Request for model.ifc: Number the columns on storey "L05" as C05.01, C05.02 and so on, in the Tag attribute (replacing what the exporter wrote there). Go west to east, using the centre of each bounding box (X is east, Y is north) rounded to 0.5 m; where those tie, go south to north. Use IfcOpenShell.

First a look at what the model holds.

```python
import ifcopenshell
import ifcopenshell.util.element
import ifcopenshell.util.placement

model = ifcopenshell.open("model.ifc")
print(model.schema)
storey = next(s for s in model.by_type("IfcBuildingStorey") if s.Name == "L05")
columns = [e for e in ifcopenshell.util.element.get_decomposition(storey) if e.is_a("IfcColumn")]
for e in sorted(columns, key=lambda e: e.id()):
    origin = ifcopenshell.util.placement.get_local_placement(e.ObjectPlacement)[:3, 3]
    print(e.id(), e.Tag, e.Name, origin.round(2) + 0.0, sep=" | ")
```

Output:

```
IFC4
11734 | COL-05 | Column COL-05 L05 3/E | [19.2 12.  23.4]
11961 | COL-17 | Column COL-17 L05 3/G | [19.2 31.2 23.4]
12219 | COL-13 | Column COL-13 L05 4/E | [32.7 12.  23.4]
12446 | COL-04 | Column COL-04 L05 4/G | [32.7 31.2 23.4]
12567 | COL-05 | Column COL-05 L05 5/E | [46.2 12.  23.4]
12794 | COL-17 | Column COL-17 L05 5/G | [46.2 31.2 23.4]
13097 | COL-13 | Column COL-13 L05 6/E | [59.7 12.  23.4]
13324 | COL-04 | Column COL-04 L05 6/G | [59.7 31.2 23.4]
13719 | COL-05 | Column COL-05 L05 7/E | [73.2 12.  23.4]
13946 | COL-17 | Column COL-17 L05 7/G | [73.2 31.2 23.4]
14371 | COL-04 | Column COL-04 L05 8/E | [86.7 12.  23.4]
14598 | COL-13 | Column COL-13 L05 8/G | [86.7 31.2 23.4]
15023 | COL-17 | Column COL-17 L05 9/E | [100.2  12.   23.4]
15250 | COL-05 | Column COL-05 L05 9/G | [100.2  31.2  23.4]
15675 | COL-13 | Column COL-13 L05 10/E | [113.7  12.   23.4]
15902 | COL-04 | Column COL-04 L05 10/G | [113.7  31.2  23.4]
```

```python
import ifcopenshell
import ifcopenshell.geom
import ifcopenshell.util.element
import ifcopenshell.util.shape

model = ifcopenshell.open("model.ifc")
settings = ifcopenshell.geom.settings()
settings.set("use-world-coords", True)


def centre(element):
    shape = ifcopenshell.geom.create_shape(settings, element)
    return ifcopenshell.util.shape.get_bbox_centroid(shape.geometry)


storey = next(s for s in model.by_type("IfcBuildingStorey") if s.Name == "L05")
columns = [e for e in ifcopenshell.util.element.get_decomposition(storey) if e.is_a("IfcColumn")]

# Insertion points can sit at a corner or the storey origin, so sort by the geometry (in metres).
centres = {e: centre(e) for e in columns}
columns.sort(key=lambda e: (round(centres[e][0] / 0.5), centres[e][1]))

for i, e in enumerate(columns, start=1):
    number = f"C05.{i:02d}"
    e.Tag = number
    print(e.id(), number)

model.write("model-out.ifc")
```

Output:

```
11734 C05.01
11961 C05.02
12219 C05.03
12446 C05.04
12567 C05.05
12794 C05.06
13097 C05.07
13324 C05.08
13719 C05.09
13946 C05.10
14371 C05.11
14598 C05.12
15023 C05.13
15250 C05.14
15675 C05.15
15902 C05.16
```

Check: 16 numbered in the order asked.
